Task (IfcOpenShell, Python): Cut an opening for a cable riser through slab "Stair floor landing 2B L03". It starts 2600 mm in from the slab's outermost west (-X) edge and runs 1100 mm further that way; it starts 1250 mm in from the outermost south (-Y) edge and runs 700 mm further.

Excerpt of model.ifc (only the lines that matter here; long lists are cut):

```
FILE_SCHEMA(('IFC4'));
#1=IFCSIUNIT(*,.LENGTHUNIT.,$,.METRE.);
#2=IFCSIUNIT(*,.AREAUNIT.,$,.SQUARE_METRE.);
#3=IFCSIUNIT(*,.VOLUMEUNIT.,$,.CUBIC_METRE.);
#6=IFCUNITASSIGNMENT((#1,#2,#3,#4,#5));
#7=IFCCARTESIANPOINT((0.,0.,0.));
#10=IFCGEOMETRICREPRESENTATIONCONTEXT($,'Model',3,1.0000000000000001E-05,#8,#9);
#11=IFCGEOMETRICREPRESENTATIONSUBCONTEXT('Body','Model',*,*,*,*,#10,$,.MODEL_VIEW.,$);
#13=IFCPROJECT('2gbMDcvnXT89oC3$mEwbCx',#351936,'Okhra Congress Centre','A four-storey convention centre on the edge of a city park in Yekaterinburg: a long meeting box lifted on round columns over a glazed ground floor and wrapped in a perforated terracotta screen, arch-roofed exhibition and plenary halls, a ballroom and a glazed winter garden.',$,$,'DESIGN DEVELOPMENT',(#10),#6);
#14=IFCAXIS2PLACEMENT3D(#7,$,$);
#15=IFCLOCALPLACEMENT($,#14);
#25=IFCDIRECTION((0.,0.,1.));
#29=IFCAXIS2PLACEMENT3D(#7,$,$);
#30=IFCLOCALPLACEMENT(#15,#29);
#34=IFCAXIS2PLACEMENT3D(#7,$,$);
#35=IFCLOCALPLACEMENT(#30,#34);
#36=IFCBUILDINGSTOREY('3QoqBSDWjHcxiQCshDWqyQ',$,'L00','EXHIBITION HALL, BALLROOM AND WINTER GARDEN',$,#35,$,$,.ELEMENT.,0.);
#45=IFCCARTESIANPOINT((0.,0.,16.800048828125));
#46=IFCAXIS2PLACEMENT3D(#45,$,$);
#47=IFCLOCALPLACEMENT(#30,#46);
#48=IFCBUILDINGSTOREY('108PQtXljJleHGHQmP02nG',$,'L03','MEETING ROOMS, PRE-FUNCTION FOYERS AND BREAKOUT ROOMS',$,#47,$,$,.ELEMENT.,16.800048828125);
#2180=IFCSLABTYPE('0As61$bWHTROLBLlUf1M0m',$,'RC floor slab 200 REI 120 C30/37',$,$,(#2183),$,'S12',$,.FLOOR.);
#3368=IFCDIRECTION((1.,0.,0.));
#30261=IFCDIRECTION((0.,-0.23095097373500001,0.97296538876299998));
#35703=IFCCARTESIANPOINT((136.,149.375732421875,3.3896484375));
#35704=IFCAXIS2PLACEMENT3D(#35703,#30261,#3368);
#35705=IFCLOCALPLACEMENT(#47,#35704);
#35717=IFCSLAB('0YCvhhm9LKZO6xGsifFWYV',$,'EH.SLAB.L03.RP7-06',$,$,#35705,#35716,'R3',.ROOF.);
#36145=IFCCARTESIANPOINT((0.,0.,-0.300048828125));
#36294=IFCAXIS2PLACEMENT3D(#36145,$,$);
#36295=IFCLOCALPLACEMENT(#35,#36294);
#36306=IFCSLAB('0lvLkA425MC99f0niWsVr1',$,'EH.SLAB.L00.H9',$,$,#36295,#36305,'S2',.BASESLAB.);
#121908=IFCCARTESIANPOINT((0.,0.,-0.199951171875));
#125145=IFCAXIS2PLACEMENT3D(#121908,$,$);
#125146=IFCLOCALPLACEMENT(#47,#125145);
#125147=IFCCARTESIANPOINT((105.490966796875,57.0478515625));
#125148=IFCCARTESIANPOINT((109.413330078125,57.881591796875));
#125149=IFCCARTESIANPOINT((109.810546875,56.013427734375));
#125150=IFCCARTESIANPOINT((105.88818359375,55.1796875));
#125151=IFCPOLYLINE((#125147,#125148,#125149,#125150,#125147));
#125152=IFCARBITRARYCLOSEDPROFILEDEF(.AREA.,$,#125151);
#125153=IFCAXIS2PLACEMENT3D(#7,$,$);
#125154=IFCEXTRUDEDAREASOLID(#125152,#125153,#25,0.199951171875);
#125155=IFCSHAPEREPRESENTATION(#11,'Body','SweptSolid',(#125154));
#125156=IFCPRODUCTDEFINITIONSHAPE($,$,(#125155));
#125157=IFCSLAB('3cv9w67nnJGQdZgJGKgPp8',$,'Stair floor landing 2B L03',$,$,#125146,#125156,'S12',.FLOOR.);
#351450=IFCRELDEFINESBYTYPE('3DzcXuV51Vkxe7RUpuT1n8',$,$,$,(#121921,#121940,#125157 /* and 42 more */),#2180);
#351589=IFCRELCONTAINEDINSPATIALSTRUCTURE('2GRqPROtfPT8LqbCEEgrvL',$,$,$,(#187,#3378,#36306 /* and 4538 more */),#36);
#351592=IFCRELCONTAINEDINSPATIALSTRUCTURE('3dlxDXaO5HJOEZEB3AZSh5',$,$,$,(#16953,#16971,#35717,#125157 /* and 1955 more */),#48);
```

```python
import numpy as np
import ifcopenshell
import ifcopenshell.api.feature
import ifcopenshell.api.geometry
import ifcopenshell.api.root
import ifcopenshell.geom
import ifcopenshell.util.placement
import ifcopenshell.util.representation
import ifcopenshell.util.shape
import ifcopenshell.util.unit

model = ifcopenshell.open("model.ifc")
unit_scale = ifcopenshell.util.unit.calculate_unit_scale(model)
settings = ifcopenshell.geom.settings()


def volume(element):
    """Net volume in cubic metres, openings subtracted."""
    shape = ifcopenshell.geom.create_shape(settings, element)
    return ifcopenshell.util.shape.get_volume(shape.geometry)


slab = model.by_guid("3cv9w67nnJGQdZgJGKgPp8")
before = volume(slab)

# Extent in the slab's own axes, in metres. The edges named are its -X and -Y sides.
slab_shape = ifcopenshell.geom.create_shape(settings, slab)
vertices = ifcopenshell.util.shape.get_vertices(slab_shape.geometry)
x_min, y_min, bottom = vertices.min(axis=0)
top = vertices[:, 2].max()

opening = ifcopenshell.api.root.create_entity(model, ifc_class="IfcOpeningElement", name="Cable riser opening", predefined_type="OPENING")
context = ifcopenshell.util.representation.get_context(model, "Model", "Body", "MODEL_VIEW")
width, depth = 1.1, 0.7
outline = [(0.0, 0.0), (width, 0.0), (width, depth), (0.0, depth), (0.0, 0.0)]
# Overshoot both faces by 50 mm so the cut is clean.
shape = ifcopenshell.api.geometry.add_slab_representation(
    model, context=context, depth=top - bottom + 0.1, polyline=outline
)
ifcopenshell.api.geometry.assign_representation(model, product=opening, representation=shape)

matrix = ifcopenshell.util.placement.get_local_placement(slab.ObjectPlacement)
matrix[:, 3] = matrix @ np.append(np.array([x_min + 2.6, y_min + 1.25, bottom - 0.05]) / unit_scale, 1.0)
ifcopenshell.api.geometry.edit_object_placement(model, product=opening, matrix=matrix, is_si=False)
ifcopenshell.api.feature.add_feature(model, feature=opening, element=slab)

after = volume(slab)

print(f"slab volume {before:.3f} -> {after:.3f} m3")

model.write("model_rev.ifc")
```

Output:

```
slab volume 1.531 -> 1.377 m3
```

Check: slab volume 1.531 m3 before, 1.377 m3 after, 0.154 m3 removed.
